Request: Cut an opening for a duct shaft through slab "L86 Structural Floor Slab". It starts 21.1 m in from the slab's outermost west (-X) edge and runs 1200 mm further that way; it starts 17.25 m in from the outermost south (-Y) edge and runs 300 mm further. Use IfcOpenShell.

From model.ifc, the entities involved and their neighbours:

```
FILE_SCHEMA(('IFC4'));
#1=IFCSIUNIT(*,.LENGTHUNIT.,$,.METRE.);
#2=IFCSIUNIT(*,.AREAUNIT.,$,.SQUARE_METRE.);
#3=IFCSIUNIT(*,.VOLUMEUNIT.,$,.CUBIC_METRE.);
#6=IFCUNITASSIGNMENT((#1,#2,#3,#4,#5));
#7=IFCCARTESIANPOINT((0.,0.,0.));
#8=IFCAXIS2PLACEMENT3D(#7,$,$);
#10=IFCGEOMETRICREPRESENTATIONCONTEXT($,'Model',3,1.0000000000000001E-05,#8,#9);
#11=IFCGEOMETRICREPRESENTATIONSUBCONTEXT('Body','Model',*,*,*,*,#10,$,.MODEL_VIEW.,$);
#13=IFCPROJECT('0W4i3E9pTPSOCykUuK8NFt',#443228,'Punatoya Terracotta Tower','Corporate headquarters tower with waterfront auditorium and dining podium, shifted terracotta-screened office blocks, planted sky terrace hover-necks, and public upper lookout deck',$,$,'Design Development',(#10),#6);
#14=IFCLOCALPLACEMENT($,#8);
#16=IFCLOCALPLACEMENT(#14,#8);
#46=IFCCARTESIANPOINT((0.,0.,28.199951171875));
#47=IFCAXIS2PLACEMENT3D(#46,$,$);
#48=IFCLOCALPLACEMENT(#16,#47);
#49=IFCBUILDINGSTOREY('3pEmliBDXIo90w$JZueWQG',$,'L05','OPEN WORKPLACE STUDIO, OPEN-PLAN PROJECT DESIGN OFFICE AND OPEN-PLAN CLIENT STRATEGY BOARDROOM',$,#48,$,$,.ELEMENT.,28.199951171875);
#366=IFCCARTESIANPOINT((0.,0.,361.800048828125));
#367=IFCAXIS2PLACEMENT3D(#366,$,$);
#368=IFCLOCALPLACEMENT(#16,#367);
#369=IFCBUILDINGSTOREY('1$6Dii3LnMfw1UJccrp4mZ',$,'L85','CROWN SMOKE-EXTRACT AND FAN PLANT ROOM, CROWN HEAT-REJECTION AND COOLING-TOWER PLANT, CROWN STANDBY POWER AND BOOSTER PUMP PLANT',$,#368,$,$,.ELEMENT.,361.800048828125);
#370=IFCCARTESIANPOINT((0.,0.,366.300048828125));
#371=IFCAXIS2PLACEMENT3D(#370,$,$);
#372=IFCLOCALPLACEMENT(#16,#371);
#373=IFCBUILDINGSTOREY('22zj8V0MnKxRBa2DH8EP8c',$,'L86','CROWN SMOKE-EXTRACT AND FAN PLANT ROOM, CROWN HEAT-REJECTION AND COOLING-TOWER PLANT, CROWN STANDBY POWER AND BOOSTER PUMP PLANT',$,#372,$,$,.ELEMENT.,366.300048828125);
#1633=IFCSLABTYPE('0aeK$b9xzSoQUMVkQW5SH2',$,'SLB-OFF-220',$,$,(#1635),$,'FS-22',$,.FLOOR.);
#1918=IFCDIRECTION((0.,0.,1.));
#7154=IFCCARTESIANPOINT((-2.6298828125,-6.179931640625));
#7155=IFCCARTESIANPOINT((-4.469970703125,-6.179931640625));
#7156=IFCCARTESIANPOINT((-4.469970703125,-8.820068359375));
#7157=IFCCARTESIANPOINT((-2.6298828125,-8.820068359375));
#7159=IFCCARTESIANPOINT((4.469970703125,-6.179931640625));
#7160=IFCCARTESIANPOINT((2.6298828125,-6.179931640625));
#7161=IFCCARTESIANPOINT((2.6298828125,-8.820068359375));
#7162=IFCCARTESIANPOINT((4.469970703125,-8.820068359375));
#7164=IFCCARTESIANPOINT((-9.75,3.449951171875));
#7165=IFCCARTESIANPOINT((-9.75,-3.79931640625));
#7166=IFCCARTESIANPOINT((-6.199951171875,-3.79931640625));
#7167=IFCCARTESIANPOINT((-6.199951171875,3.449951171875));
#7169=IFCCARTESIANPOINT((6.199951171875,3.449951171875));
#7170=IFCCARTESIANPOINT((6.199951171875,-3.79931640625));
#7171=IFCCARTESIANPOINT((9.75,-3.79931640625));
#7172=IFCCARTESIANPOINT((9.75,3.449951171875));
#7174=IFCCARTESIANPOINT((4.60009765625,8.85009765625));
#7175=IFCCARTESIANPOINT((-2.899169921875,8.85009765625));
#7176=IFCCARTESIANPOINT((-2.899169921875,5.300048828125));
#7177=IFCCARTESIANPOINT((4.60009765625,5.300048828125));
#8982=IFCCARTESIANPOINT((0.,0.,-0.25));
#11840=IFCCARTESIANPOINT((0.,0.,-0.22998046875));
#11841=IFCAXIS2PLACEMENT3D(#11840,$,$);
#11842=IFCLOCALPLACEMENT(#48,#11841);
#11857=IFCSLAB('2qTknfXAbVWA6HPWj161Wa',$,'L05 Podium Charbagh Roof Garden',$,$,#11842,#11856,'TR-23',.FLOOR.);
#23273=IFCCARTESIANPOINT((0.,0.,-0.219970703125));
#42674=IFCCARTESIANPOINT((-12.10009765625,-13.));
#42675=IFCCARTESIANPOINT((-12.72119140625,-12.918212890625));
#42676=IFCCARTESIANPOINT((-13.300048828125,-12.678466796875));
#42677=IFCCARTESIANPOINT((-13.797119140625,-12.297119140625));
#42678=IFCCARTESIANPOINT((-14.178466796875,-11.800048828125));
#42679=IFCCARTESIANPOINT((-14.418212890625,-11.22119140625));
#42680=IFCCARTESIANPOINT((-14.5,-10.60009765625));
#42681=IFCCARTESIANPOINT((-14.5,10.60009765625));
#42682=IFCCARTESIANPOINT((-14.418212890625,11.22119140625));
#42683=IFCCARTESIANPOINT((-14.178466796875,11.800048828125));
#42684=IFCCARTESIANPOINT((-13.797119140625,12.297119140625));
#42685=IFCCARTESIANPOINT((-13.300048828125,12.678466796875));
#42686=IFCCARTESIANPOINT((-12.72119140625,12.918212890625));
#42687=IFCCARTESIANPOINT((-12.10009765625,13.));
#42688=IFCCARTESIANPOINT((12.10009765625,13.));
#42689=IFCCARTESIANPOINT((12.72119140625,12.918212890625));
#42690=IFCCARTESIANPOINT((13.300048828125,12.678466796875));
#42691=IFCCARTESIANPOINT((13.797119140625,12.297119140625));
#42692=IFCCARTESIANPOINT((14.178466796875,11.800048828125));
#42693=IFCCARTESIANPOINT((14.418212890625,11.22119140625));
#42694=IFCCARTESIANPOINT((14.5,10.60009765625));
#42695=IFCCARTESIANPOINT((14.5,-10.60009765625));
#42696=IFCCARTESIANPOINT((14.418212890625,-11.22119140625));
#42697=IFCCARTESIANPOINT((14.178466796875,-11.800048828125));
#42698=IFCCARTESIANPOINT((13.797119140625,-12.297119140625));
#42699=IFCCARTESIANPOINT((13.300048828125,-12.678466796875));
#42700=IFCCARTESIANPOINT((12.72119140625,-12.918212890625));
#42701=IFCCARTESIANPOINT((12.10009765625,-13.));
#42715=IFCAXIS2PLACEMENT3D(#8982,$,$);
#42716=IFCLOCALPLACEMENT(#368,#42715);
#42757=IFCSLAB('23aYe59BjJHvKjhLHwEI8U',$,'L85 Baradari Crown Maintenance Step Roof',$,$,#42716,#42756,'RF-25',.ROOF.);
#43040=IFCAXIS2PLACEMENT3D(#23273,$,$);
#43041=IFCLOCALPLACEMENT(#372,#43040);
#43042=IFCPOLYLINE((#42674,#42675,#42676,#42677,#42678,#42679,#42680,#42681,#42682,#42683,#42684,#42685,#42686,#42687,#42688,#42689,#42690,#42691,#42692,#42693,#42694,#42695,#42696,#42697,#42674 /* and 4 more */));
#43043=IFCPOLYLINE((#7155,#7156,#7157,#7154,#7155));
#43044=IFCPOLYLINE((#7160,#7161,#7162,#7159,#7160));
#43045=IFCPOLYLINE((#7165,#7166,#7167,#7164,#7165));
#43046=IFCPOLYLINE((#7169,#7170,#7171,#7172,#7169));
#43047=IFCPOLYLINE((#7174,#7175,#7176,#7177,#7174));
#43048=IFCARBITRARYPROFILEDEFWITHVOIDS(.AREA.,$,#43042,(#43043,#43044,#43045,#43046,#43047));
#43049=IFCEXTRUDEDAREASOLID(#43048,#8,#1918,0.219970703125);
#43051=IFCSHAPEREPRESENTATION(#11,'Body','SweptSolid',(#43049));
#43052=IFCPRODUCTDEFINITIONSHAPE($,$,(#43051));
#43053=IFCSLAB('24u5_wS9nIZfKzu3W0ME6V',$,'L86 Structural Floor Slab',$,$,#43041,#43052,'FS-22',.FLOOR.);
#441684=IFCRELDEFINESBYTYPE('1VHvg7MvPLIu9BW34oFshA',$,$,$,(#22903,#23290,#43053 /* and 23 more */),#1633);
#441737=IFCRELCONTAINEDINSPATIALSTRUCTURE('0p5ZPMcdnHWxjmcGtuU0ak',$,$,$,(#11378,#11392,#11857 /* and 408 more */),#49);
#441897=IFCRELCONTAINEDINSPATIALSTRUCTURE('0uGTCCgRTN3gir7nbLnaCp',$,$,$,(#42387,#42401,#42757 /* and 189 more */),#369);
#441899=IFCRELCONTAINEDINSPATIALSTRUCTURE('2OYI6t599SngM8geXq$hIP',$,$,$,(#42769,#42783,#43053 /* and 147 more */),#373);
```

```python
import numpy as np
import ifcopenshell
import ifcopenshell.api.feature
import ifcopenshell.api.geometry
import ifcopenshell.api.root
import ifcopenshell.geom
import ifcopenshell.util.placement
import ifcopenshell.util.representation
import ifcopenshell.util.shape
import ifcopenshell.util.unit

model = ifcopenshell.open("model.ifc")
unit_scale = ifcopenshell.util.unit.calculate_unit_scale(model)
settings = ifcopenshell.geom.settings()


def volume(element):
    """Net volume in cubic metres, openings subtracted."""
    shape = ifcopenshell.geom.create_shape(settings, element)
    return ifcopenshell.util.shape.get_volume(shape.geometry)


slab = model.by_guid("24u5_wS9nIZfKzu3W0ME6V")
before = volume(slab)

# Extent in the slab's own axes, in metres. The edges named are its -X and -Y sides.
slab_shape = ifcopenshell.geom.create_shape(settings, slab)
vertices = ifcopenshell.util.shape.get_vertices(slab_shape.geometry)
x_min, y_min, bottom = vertices.min(axis=0)
top = vertices[:, 2].max()

opening = ifcopenshell.api.root.create_entity(model, ifc_class="IfcOpeningElement", name="Duct shaft opening", predefined_type="OPENING")
context = ifcopenshell.util.representation.get_context(model, "Model", "Body", "MODEL_VIEW")
width, depth = 1.2, 0.3
outline = [(0.0, 0.0), (width, 0.0), (width, depth), (0.0, depth), (0.0, 0.0)]
# Overshoot both faces by 50 mm so the cut is clean.
shape = ifcopenshell.api.geometry.add_slab_representation(
    model, context=context, depth=top - bottom + 0.1, polyline=outline
)
ifcopenshell.api.geometry.assign_representation(model, product=opening, representation=shape)

matrix = ifcopenshell.util.placement.get_local_placement(slab.ObjectPlacement)
matrix[:, 3] = matrix @ np.append(np.array([x_min + 21.1, y_min + 17.25, bottom - 0.05]) / unit_scale, 1.0)
ifcopenshell.api.geometry.edit_object_placement(model, product=opening, matrix=matrix, is_si=False)
ifcopenshell.api.feature.add_feature(model, feature=opening, element=slab)

after = volume(slab)

print(f"slab volume {before:.3f} -> {after:.3f} m3")

model.write("model_v2.ifc")
```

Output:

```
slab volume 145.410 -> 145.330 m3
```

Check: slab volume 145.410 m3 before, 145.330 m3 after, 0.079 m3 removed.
